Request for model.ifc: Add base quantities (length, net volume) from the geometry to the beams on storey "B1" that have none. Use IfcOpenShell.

First a look at what the model holds.

```python
import ifcopenshell
import ifcopenshell.util.element
import ifcopenshell.util.unit

model = ifcopenshell.open("model.ifc")
print(model.schema)
for unit_type in ("LENGTHUNIT", "AREAUNIT", "VOLUMEUNIT"):
    print(unit_type, ifcopenshell.util.unit.calculate_unit_scale(model, unit_type))
storey = next(s for s in model.by_type("IfcBuildingStorey") if s.Name == "B1")
beams = [e for e in ifcopenshell.util.element.get_decomposition(storey) if e.is_a("IfcBeam")]
for e in sorted(beams, key=lambda e: e.id()):
    print(e.id(), e.is_a(), e.Name, list(ifcopenshell.util.element.get_psets(e, qtos_only=True)), sep=" | ")
```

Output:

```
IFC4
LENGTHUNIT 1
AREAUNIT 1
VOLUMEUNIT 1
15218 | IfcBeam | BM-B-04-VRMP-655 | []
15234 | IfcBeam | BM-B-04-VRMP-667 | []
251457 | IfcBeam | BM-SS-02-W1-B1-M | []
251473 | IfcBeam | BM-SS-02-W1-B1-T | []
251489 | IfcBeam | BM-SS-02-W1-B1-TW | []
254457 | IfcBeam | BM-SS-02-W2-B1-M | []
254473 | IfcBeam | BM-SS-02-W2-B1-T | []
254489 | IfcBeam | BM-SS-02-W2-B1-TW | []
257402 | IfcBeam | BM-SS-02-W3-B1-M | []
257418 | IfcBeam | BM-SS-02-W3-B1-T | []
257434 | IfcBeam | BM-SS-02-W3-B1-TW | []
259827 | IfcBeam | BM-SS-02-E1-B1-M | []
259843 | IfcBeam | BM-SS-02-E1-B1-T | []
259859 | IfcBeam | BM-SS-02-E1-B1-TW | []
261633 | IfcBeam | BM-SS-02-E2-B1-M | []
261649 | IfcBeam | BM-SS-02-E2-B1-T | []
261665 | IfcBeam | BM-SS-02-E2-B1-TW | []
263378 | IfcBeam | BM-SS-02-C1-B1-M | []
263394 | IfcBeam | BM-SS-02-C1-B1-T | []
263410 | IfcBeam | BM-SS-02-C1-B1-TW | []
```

```python
import ifcopenshell
import ifcopenshell.api.pset
import ifcopenshell.geom
import ifcopenshell.util.element
import ifcopenshell.util.shape
import ifcopenshell.util.unit

model = ifcopenshell.open("model.ifc")
unit_scale = ifcopenshell.util.unit.calculate_unit_scale(model)
volume_scale = ifcopenshell.util.unit.calculate_unit_scale(model, "VOLUMEUNIT")
settings = ifcopenshell.geom.settings()

storey = next(s for s in model.by_type("IfcBuildingStorey") if s.Name == "B1")
beams = [e for e in ifcopenshell.util.element.get_decomposition(storey) if e.is_a("IfcBeam")]

for e in sorted(beams, key=lambda e: e.id()):
    if ifcopenshell.util.element.get_psets(e, qtos_only=True, should_inherit=False):
        continue
    # Geometry comes back in metres, in the element's own axes.
    shape = ifcopenshell.geom.create_shape(settings, e)
    values = {
        "Length": ifcopenshell.util.shape.get_max_xyz(shape.geometry) / unit_scale,
        "NetVolume": ifcopenshell.util.shape.get_volume(shape.geometry) / volume_scale,
    }
    qto = ifcopenshell.api.pset.add_qto(model, product=e, name="Qto_BeamBaseQuantities")
    ifcopenshell.api.pset.edit_qto(model, qto=qto, properties=values)
    print(e.id(), {k: round(v, 3) for k, v in values.items()})

model.write("model_updated.ifc")
```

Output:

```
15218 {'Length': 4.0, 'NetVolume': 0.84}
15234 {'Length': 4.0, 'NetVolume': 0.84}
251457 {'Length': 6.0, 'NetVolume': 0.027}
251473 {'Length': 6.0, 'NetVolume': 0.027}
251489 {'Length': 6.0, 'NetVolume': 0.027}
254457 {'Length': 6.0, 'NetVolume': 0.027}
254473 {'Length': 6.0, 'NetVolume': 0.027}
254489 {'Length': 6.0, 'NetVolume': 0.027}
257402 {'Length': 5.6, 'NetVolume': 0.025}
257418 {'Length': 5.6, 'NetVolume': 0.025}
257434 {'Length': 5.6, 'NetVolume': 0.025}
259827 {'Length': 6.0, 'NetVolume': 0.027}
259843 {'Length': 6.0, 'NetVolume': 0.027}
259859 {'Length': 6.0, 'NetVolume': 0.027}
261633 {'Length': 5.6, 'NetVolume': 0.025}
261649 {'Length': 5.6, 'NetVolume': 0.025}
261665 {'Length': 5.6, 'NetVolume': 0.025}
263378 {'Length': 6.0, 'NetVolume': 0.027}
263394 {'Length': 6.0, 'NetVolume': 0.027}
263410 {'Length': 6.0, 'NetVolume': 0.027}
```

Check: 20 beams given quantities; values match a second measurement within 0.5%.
